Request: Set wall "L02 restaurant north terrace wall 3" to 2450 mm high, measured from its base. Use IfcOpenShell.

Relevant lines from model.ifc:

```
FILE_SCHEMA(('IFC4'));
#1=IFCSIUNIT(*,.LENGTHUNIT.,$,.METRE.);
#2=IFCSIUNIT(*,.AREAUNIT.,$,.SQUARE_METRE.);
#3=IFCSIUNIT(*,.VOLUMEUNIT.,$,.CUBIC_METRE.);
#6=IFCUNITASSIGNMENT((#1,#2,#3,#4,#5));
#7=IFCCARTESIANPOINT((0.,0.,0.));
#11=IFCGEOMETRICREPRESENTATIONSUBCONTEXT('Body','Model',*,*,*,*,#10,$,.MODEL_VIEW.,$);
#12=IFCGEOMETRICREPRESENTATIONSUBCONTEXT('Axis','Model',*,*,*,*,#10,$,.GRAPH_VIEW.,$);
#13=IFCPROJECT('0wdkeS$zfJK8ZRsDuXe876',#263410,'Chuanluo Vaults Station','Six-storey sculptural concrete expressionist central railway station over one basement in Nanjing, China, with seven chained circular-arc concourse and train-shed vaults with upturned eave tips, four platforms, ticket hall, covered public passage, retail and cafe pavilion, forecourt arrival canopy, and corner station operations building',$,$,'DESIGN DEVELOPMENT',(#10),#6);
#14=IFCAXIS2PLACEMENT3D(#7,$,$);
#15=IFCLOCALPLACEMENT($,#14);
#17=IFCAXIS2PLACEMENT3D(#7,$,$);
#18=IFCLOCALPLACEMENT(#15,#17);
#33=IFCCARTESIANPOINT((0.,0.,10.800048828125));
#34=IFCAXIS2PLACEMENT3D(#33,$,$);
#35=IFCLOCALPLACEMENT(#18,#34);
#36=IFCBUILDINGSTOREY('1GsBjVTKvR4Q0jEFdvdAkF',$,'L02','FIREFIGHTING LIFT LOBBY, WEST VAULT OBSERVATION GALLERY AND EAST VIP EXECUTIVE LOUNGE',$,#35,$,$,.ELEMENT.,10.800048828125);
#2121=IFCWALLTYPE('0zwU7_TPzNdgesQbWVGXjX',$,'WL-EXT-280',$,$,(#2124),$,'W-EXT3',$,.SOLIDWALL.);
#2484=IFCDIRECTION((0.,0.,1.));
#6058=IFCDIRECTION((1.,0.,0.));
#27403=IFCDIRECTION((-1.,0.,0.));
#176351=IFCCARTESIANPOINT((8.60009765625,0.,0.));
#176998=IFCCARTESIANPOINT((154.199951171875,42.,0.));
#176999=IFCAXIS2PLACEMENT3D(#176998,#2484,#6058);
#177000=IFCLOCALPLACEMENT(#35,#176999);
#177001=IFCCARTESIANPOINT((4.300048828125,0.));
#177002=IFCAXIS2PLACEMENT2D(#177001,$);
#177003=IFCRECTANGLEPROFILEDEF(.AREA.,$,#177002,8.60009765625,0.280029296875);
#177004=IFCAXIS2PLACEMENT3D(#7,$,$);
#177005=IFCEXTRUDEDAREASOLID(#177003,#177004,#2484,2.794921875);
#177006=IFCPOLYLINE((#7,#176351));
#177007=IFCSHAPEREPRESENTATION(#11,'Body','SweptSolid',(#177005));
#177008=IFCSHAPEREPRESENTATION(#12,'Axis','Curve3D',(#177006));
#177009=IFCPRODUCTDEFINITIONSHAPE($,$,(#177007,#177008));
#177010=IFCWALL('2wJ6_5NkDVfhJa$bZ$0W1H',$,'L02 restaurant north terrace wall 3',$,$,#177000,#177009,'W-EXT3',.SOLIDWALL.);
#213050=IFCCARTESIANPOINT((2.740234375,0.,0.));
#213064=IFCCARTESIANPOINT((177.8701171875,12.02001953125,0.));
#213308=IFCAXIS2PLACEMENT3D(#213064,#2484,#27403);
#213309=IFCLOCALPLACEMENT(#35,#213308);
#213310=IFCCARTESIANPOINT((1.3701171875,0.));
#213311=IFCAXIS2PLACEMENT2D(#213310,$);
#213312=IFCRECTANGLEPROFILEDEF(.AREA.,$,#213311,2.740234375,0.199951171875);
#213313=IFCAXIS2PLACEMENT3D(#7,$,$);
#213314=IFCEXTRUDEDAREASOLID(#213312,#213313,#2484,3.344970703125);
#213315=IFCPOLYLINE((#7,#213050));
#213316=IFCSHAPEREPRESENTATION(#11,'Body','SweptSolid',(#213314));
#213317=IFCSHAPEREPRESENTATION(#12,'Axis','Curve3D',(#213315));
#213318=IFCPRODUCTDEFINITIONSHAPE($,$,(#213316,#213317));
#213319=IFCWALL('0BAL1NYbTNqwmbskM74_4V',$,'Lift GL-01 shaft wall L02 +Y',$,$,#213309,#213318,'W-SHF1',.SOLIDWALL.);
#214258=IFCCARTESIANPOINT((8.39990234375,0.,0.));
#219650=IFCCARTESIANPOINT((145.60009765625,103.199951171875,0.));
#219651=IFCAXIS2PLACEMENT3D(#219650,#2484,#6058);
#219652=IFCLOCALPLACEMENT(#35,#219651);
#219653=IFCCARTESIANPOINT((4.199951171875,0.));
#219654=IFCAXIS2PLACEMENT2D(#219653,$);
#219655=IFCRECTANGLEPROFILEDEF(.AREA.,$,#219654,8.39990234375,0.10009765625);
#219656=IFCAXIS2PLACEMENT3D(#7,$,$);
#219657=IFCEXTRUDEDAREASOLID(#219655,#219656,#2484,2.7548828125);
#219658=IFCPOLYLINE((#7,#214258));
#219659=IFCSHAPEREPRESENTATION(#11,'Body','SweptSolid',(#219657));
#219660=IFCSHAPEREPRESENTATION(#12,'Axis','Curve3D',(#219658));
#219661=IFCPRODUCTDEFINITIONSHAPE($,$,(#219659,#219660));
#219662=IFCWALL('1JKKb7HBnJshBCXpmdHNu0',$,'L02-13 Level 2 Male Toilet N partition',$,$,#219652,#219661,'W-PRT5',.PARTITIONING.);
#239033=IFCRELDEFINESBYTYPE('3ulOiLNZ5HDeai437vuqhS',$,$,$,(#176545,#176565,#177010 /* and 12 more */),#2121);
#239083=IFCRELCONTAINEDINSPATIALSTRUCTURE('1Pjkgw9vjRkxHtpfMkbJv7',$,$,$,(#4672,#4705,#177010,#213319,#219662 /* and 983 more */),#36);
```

```python
import ifcopenshell
import ifcopenshell.geom
import ifcopenshell.util.representation
import ifcopenshell.util.shape
import ifcopenshell.util.unit

model = ifcopenshell.open("model.ifc")
unit_scale = ifcopenshell.util.unit.calculate_unit_scale(model)
settings = ifcopenshell.geom.settings()


def volume(element):
    """Net volume in cubic metres, openings subtracted."""
    shape = ifcopenshell.geom.create_shape(settings, element)
    return ifcopenshell.util.shape.get_volume(shape.geometry)


wall = model.by_guid("2wJ6_5NkDVfhJa$bZ$0W1H")
before = volume(wall)

body = ifcopenshell.util.representation.get_representation(wall, "Model", "Body")
solid = body.Items[0]
old_height = solid.Depth
solid.Depth = 2.45 / unit_scale
after = volume(wall)

print(f"height {old_height:g} -> {solid.Depth:g}, volume {before:.3f} -> {after:.3f} m3")

model.write("model_v2.ifc")
```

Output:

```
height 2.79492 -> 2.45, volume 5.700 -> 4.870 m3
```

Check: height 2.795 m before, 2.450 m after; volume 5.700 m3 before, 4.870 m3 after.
